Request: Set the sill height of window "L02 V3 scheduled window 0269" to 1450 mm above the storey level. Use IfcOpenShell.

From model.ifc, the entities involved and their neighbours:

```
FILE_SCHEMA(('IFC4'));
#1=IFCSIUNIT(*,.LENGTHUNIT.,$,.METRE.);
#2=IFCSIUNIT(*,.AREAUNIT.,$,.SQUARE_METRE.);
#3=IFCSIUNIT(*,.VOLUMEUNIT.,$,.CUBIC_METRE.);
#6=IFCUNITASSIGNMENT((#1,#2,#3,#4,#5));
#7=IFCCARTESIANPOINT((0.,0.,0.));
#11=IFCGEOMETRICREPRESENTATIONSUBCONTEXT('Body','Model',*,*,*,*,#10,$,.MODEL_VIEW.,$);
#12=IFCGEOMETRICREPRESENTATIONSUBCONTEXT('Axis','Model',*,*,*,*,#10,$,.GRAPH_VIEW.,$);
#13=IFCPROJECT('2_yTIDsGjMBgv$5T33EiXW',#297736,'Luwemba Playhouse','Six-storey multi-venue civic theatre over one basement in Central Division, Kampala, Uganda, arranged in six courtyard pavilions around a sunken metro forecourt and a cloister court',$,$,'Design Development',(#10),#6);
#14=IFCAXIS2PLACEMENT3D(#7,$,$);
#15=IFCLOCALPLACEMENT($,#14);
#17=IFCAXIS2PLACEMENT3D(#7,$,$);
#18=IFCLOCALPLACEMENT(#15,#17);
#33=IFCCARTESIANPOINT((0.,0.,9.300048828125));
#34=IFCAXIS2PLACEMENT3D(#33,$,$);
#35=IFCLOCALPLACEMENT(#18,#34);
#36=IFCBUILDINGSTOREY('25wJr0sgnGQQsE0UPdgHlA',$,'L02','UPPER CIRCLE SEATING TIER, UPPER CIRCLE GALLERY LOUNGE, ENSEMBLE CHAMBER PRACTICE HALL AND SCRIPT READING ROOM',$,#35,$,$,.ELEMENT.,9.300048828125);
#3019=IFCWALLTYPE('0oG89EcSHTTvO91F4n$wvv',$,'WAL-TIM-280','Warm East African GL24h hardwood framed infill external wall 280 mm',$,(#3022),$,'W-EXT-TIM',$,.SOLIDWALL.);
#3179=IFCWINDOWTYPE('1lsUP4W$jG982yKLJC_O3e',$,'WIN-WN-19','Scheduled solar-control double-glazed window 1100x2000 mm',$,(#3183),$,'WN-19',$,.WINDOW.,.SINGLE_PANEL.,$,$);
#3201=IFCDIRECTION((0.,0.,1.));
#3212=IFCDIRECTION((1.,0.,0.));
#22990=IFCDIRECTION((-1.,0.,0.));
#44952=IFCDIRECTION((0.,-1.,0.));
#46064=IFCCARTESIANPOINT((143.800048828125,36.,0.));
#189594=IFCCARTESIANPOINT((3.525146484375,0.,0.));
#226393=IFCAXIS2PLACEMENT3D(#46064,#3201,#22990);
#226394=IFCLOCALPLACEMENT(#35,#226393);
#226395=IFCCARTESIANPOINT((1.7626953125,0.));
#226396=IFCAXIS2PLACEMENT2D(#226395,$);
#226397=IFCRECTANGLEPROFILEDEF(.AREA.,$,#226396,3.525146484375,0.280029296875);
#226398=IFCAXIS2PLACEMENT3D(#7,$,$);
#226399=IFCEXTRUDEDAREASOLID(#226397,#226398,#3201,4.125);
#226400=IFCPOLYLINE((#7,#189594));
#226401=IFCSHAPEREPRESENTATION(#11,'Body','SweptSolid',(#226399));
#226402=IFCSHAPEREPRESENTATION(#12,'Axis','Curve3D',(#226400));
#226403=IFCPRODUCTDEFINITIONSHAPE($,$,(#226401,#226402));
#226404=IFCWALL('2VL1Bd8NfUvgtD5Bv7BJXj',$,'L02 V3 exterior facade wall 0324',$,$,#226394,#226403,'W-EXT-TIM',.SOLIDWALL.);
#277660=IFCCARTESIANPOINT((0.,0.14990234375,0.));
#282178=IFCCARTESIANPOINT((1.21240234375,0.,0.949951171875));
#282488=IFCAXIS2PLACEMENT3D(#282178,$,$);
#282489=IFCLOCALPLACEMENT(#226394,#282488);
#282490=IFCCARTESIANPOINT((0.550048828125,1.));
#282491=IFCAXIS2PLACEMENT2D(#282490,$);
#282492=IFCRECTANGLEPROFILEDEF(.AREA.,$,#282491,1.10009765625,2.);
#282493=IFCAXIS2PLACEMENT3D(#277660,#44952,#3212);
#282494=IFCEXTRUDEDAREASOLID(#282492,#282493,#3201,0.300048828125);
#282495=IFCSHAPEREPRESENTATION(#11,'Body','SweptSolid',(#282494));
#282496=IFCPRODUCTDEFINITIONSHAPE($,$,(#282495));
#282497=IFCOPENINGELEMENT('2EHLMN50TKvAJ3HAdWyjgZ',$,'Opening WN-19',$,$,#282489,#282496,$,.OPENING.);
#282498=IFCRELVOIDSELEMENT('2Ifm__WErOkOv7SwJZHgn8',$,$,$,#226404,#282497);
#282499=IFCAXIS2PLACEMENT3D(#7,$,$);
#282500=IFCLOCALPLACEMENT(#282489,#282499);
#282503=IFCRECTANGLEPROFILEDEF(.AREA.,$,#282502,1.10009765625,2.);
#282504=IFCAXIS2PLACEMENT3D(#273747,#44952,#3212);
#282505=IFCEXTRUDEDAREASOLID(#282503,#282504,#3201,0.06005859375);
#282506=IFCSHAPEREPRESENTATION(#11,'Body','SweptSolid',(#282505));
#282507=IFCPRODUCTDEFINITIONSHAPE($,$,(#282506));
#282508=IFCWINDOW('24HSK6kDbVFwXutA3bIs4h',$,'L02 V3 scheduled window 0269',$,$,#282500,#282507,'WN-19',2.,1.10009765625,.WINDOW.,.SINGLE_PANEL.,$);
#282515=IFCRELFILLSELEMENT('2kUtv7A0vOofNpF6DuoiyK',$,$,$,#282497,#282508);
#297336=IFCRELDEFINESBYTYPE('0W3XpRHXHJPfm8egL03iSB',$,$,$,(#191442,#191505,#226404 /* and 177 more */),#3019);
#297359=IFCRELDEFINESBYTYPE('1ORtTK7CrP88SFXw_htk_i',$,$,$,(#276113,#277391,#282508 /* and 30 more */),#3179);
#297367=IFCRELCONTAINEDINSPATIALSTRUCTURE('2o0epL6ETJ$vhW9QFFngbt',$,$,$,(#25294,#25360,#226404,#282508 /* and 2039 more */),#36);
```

```python
import numpy as np
import ifcopenshell
import ifcopenshell.api.geometry
import ifcopenshell.geom
import ifcopenshell.util.element
import ifcopenshell.util.placement
import ifcopenshell.util.shape
import ifcopenshell.util.unit

model = ifcopenshell.open("model.ifc")
unit_scale = ifcopenshell.util.unit.calculate_unit_scale(model)

window = model.by_id(282508)
opening = window.FillsVoids[0].RelatingOpeningElement
storey = ifcopenshell.util.element.get_container(window, ifc_class="IfcBuildingStorey")
level = ifcopenshell.util.placement.get_local_placement(storey.ObjectPlacement)[2, 3]

# The opening's origin need not be at the sill, so measure its lowest point.
shape = ifcopenshell.geom.create_shape(ifcopenshell.geom.settings(), opening)
bottom = ifcopenshell.util.shape.get_shape_bottom_elevation(shape, shape.geometry) / unit_scale
dz = level + 1.45 - bottom

shift = np.array([0.0, 0.0, dz])
# The window is placed relative to its opening, so it follows when the opening moves.
matrix = ifcopenshell.util.placement.get_local_placement(opening.ObjectPlacement)
matrix[:3, 3] += shift
ifcopenshell.api.geometry.edit_object_placement(
    model, product=opening, matrix=matrix, is_si=False, should_transform_children=True
)

print(f"moved by {dz * unit_scale:+.3f} m")

model.write("model_v2.ifc")
```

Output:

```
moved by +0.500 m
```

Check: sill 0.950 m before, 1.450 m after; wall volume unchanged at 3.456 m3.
